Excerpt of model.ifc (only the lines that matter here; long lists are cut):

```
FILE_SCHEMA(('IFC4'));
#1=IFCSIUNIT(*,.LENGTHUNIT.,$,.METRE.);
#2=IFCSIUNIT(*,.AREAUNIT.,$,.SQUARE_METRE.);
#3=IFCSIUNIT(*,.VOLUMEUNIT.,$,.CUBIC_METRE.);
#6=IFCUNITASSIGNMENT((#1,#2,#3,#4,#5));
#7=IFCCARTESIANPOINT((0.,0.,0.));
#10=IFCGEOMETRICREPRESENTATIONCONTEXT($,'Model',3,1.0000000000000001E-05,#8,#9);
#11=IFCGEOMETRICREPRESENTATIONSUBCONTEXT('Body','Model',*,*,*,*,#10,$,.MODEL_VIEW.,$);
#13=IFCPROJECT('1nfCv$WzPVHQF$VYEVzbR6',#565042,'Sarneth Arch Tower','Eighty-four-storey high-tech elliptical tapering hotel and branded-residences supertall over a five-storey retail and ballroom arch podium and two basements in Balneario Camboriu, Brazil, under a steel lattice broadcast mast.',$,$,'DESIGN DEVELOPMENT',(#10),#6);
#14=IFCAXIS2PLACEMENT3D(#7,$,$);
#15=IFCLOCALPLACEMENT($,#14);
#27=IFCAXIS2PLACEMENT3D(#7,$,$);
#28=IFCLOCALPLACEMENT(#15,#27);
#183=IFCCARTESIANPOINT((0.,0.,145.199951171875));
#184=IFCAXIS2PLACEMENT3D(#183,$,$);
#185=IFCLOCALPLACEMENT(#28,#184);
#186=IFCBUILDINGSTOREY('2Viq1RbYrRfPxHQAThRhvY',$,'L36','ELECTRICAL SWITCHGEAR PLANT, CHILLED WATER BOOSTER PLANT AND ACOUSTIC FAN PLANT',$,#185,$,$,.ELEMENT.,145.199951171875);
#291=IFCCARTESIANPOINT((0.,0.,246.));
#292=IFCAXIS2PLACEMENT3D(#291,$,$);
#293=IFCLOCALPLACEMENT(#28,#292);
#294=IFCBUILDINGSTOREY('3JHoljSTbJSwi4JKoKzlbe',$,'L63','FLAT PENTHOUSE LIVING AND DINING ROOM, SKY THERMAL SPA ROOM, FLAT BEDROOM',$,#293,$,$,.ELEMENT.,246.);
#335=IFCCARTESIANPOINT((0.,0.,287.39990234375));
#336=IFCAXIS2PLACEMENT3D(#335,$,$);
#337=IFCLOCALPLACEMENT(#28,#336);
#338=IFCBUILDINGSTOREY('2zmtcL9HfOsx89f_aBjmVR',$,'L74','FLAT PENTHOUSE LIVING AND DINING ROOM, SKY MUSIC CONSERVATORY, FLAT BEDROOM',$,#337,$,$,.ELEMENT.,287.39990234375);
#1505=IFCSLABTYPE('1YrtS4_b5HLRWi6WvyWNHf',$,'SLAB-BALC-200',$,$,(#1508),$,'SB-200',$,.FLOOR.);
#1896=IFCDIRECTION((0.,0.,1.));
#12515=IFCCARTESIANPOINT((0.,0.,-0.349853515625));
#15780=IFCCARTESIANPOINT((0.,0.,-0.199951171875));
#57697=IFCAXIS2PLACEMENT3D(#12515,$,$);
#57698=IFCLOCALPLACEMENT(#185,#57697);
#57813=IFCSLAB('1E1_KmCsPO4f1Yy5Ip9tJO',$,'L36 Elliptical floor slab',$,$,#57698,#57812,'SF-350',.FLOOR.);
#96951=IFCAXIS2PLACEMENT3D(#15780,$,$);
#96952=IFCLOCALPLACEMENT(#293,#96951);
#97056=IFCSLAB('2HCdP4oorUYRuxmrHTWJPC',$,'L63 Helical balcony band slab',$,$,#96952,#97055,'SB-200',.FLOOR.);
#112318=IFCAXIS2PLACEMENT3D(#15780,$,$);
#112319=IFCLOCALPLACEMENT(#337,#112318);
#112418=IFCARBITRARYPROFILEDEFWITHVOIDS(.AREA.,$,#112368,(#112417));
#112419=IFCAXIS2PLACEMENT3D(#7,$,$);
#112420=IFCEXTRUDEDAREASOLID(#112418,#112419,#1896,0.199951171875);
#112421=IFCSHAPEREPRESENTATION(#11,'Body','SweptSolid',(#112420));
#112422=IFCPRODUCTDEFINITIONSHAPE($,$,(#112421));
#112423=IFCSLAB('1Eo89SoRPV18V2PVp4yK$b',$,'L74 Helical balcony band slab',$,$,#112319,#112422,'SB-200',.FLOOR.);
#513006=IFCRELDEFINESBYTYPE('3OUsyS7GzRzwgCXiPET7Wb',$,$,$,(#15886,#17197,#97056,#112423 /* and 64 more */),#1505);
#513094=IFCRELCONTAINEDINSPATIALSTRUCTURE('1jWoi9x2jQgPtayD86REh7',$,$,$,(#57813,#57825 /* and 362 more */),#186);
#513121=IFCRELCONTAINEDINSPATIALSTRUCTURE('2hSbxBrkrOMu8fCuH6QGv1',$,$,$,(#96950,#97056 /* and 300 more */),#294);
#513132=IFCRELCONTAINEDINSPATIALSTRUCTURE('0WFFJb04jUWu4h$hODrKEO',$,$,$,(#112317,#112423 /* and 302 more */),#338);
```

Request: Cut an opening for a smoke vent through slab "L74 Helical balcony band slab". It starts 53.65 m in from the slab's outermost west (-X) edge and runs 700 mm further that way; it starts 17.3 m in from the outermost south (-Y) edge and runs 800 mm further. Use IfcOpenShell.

```python
import numpy as np
import ifcopenshell
import ifcopenshell.api.feature
import ifcopenshell.api.geometry
import ifcopenshell.api.root
import ifcopenshell.geom
import ifcopenshell.util.placement
import ifcopenshell.util.representation
import ifcopenshell.util.shape
import ifcopenshell.util.unit

model = ifcopenshell.open("model.ifc")
unit_scale = ifcopenshell.util.unit.calculate_unit_scale(model)
settings = ifcopenshell.geom.settings()


def volume(element):
    """Net volume in cubic metres, openings subtracted."""
    shape = ifcopenshell.geom.create_shape(settings, element)
    return ifcopenshell.util.shape.get_volume(shape.geometry)


slab = model.by_id(112423)
before = volume(slab)

# Extent in the slab's own axes, in metres. The edges named are its -X and -Y sides.
slab_shape = ifcopenshell.geom.create_shape(settings, slab)
vertices = ifcopenshell.util.shape.get_vertices(slab_shape.geometry)
x_min, y_min, bottom = vertices.min(axis=0)
top = vertices[:, 2].max()

opening = ifcopenshell.api.root.create_entity(model, ifc_class="IfcOpeningElement", name="Smoke vent opening", predefined_type="OPENING")
context = ifcopenshell.util.representation.get_context(model, "Model", "Body", "MODEL_VIEW")
width, depth = 0.7, 0.8
outline = [(0.0, 0.0), (width, 0.0), (width, depth), (0.0, depth), (0.0, 0.0)]
# Overshoot both faces by 50 mm so the cut is clean.
shape = ifcopenshell.api.geometry.add_slab_representation(
    model, context=context, depth=top - bottom + 0.1, polyline=outline
)
ifcopenshell.api.geometry.assign_representation(model, product=opening, representation=shape)

matrix = ifcopenshell.util.placement.get_local_placement(slab.ObjectPlacement)
matrix[:, 3] = matrix @ np.append(np.array([x_min + 53.65, y_min + 17.3, bottom - 0.05]) / unit_scale, 1.0)
ifcopenshell.api.geometry.edit_object_placement(model, product=opening, matrix=matrix, is_si=False)
ifcopenshell.api.feature.add_feature(model, feature=opening, element=slab)

after = volume(slab)

print(f"slab volume {before:.3f} -> {after:.3f} m3")

model.write("model_v2.ifc")
```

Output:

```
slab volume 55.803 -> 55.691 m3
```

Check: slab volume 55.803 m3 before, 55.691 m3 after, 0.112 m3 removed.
